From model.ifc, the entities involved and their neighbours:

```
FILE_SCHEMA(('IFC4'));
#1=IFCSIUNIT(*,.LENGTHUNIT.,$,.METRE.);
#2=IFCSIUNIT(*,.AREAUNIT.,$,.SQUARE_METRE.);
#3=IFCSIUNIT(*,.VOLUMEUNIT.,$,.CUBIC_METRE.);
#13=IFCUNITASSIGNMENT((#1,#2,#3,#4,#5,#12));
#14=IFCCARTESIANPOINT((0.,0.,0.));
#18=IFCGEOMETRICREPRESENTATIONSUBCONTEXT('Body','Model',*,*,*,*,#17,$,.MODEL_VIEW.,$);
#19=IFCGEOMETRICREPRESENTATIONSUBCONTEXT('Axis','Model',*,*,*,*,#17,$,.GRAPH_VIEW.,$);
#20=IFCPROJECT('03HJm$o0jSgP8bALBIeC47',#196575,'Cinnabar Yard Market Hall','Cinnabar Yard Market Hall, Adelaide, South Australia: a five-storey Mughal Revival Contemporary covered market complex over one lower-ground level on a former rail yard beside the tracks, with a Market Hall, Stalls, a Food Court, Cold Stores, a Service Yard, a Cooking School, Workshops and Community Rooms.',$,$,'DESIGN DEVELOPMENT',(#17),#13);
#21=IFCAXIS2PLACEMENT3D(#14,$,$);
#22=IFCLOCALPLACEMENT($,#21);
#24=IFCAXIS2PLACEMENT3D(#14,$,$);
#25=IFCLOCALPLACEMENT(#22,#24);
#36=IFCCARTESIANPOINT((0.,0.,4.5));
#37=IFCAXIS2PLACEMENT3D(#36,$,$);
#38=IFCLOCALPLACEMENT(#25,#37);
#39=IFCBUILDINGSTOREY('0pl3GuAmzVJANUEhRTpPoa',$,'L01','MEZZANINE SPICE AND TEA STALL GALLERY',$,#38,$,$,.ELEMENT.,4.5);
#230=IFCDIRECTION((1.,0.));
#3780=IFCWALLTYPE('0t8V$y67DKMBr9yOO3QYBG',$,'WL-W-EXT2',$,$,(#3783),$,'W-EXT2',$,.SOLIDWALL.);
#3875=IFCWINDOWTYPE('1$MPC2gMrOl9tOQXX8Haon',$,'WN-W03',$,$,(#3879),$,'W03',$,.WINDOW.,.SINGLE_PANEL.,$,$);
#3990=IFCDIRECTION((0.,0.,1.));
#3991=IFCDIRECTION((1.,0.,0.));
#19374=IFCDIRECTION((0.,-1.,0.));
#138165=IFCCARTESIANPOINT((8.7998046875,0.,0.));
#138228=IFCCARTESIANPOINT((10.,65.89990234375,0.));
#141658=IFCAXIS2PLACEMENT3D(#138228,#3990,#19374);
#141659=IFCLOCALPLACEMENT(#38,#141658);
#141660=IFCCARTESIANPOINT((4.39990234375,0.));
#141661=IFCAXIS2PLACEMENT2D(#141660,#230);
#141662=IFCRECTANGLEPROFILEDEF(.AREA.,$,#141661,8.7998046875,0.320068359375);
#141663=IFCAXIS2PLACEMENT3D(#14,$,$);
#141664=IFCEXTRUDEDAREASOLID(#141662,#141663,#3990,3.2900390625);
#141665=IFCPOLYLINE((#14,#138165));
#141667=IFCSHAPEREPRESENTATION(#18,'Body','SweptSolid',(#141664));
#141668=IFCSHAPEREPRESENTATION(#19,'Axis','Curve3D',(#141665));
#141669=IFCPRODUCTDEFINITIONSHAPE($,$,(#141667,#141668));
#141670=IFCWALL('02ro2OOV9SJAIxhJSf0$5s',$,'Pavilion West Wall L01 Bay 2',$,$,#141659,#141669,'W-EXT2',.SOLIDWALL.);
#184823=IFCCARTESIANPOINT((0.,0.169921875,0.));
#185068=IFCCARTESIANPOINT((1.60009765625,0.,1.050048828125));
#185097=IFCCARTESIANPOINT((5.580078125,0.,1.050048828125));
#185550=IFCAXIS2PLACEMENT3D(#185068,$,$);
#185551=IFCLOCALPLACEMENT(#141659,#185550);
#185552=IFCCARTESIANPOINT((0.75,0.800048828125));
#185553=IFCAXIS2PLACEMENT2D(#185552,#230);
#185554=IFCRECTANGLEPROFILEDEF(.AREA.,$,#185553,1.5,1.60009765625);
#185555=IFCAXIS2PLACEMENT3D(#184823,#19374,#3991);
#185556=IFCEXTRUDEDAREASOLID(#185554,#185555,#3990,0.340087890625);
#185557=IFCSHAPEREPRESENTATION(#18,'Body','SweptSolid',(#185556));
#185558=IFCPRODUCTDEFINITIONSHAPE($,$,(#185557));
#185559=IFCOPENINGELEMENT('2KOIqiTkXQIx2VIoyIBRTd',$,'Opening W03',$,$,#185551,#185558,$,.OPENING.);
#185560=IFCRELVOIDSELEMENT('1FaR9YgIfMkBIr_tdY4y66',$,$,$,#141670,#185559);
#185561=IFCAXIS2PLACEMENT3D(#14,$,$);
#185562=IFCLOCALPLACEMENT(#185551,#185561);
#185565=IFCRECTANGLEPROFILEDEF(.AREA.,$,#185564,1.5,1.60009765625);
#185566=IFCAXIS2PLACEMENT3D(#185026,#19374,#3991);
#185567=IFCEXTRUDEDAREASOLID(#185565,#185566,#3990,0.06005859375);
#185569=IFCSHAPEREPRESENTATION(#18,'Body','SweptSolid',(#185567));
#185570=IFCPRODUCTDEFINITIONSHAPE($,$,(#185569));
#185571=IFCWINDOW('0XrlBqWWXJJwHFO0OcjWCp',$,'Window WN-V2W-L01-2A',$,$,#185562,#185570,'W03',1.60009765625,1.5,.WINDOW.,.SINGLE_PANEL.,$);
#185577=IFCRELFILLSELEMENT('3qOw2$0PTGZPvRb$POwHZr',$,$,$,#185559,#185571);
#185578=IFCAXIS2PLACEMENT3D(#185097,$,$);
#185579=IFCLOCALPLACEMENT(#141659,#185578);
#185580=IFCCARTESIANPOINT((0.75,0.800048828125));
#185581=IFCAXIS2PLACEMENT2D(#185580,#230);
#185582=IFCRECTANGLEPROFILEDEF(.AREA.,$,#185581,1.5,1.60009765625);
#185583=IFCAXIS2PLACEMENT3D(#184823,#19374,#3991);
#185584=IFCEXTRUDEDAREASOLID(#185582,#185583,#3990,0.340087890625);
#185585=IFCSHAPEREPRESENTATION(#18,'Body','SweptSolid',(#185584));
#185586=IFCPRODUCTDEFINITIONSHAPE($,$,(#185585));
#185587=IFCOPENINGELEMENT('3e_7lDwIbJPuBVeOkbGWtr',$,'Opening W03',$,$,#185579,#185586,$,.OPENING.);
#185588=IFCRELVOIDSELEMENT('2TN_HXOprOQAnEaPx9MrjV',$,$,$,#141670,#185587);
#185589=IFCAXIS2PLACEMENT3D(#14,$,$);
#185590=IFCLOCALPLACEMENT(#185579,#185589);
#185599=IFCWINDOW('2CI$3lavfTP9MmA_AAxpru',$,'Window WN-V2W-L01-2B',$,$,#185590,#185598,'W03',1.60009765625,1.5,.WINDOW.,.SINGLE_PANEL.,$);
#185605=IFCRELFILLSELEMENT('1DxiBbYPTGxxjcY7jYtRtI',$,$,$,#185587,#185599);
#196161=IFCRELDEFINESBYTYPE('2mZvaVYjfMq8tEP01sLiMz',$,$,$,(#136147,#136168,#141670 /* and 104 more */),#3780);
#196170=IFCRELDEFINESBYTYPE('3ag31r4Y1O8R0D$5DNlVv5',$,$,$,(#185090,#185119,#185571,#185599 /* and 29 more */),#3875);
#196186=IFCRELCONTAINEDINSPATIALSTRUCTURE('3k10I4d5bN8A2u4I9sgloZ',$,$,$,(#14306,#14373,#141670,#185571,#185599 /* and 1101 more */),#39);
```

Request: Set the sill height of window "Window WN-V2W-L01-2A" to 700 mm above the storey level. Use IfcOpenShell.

```python
import numpy as np
import ifcopenshell
import ifcopenshell.api.geometry
import ifcopenshell.geom
import ifcopenshell.util.element
import ifcopenshell.util.placement
import ifcopenshell.util.shape
import ifcopenshell.util.unit

model = ifcopenshell.open("model.ifc")
unit_scale = ifcopenshell.util.unit.calculate_unit_scale(model)

window = model.by_guid("0XrlBqWWXJJwHFO0OcjWCp")
opening = window.FillsVoids[0].RelatingOpeningElement
storey = ifcopenshell.util.element.get_container(window, ifc_class="IfcBuildingStorey")
level = ifcopenshell.util.placement.get_local_placement(storey.ObjectPlacement)[2, 3]

# The opening's origin need not be at the sill, so measure its lowest point.
shape = ifcopenshell.geom.create_shape(ifcopenshell.geom.settings(), opening)
bottom = ifcopenshell.util.shape.get_shape_bottom_elevation(shape, shape.geometry) / unit_scale
dz = level + 0.7 / unit_scale - bottom

shift = np.array([0.0, 0.0, dz])
# The window is placed relative to its opening, so it follows when the opening moves.
matrix = ifcopenshell.util.placement.get_local_placement(opening.ObjectPlacement)
matrix[:3, 3] += shift
ifcopenshell.api.geometry.edit_object_placement(
    model, product=opening, matrix=matrix, is_si=False, should_transform_children=True
)

print(f"moved by {dz * unit_scale:+.3f} m")

model.write("model_v2.ifc")
```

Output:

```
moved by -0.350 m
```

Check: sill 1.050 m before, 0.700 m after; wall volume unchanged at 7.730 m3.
